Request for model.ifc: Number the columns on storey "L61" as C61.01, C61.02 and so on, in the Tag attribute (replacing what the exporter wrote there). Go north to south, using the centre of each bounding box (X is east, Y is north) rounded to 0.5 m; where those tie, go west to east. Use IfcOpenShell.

First a look at what the model holds.

```python
import ifcopenshell
import ifcopenshell.util.element
import ifcopenshell.util.placement

model = ifcopenshell.open("model.ifc")
print(model.schema)
storey = next(s for s in model.by_type("IfcBuildingStorey") if s.Name == "L61")
columns = [e for e in ifcopenshell.util.element.get_decomposition(storey) if e.is_a("IfcColumn")]
for e in sorted(columns, key=lambda e: e.id()):
    origin = ifcopenshell.util.placement.get_local_placement(e.ObjectPlacement)[:3, 3]
    print(e.id(), e.Tag, e.Name, origin.round(2) + 0.0, sep=" | ")
```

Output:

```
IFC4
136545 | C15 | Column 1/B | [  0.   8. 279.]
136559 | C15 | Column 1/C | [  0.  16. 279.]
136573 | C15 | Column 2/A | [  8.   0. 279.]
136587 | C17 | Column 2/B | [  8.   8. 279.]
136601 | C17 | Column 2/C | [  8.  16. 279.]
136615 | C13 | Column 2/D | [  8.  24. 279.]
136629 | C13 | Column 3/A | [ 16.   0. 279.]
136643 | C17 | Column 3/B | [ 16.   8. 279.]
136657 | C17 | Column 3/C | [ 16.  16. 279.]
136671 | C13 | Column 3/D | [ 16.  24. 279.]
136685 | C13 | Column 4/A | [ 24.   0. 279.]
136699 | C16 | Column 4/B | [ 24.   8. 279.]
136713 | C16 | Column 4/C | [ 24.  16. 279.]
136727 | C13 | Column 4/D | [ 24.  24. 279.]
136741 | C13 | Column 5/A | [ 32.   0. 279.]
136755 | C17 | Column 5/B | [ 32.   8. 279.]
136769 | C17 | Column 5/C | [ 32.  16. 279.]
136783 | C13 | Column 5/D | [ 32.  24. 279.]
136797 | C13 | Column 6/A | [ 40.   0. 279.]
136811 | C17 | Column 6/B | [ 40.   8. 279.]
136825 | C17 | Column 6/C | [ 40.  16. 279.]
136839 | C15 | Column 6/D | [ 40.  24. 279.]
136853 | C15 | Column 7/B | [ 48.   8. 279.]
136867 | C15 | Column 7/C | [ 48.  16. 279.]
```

```python
import ifcopenshell
import ifcopenshell.geom
import ifcopenshell.util.element
import ifcopenshell.util.shape

model = ifcopenshell.open("model.ifc")
settings = ifcopenshell.geom.settings()
settings.set("use-world-coords", True)


def centre(element):
    shape = ifcopenshell.geom.create_shape(settings, element)
    return ifcopenshell.util.shape.get_bbox_centroid(shape.geometry)


storey = next(s for s in model.by_type("IfcBuildingStorey") if s.Name == "L61")
columns = [e for e in ifcopenshell.util.element.get_decomposition(storey) if e.is_a("IfcColumn")]

# Insertion points can sit at a corner or the storey origin, so sort by the geometry (in metres).
centres = {e: centre(e) for e in columns}
columns.sort(key=lambda e: (-round(centres[e][1] / 0.5), centres[e][0]))

for i, e in enumerate(columns, start=1):
    number = f"C61.{i:02d}"
    e.Tag = number
    print(e.id(), number)

model.write("model_rev.ifc")
```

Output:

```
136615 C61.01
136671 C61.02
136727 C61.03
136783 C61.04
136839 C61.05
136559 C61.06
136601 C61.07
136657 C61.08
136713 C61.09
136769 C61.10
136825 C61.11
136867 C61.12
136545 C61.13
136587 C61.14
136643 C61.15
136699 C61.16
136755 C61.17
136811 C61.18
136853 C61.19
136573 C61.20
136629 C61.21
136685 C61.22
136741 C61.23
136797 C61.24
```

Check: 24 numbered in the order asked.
